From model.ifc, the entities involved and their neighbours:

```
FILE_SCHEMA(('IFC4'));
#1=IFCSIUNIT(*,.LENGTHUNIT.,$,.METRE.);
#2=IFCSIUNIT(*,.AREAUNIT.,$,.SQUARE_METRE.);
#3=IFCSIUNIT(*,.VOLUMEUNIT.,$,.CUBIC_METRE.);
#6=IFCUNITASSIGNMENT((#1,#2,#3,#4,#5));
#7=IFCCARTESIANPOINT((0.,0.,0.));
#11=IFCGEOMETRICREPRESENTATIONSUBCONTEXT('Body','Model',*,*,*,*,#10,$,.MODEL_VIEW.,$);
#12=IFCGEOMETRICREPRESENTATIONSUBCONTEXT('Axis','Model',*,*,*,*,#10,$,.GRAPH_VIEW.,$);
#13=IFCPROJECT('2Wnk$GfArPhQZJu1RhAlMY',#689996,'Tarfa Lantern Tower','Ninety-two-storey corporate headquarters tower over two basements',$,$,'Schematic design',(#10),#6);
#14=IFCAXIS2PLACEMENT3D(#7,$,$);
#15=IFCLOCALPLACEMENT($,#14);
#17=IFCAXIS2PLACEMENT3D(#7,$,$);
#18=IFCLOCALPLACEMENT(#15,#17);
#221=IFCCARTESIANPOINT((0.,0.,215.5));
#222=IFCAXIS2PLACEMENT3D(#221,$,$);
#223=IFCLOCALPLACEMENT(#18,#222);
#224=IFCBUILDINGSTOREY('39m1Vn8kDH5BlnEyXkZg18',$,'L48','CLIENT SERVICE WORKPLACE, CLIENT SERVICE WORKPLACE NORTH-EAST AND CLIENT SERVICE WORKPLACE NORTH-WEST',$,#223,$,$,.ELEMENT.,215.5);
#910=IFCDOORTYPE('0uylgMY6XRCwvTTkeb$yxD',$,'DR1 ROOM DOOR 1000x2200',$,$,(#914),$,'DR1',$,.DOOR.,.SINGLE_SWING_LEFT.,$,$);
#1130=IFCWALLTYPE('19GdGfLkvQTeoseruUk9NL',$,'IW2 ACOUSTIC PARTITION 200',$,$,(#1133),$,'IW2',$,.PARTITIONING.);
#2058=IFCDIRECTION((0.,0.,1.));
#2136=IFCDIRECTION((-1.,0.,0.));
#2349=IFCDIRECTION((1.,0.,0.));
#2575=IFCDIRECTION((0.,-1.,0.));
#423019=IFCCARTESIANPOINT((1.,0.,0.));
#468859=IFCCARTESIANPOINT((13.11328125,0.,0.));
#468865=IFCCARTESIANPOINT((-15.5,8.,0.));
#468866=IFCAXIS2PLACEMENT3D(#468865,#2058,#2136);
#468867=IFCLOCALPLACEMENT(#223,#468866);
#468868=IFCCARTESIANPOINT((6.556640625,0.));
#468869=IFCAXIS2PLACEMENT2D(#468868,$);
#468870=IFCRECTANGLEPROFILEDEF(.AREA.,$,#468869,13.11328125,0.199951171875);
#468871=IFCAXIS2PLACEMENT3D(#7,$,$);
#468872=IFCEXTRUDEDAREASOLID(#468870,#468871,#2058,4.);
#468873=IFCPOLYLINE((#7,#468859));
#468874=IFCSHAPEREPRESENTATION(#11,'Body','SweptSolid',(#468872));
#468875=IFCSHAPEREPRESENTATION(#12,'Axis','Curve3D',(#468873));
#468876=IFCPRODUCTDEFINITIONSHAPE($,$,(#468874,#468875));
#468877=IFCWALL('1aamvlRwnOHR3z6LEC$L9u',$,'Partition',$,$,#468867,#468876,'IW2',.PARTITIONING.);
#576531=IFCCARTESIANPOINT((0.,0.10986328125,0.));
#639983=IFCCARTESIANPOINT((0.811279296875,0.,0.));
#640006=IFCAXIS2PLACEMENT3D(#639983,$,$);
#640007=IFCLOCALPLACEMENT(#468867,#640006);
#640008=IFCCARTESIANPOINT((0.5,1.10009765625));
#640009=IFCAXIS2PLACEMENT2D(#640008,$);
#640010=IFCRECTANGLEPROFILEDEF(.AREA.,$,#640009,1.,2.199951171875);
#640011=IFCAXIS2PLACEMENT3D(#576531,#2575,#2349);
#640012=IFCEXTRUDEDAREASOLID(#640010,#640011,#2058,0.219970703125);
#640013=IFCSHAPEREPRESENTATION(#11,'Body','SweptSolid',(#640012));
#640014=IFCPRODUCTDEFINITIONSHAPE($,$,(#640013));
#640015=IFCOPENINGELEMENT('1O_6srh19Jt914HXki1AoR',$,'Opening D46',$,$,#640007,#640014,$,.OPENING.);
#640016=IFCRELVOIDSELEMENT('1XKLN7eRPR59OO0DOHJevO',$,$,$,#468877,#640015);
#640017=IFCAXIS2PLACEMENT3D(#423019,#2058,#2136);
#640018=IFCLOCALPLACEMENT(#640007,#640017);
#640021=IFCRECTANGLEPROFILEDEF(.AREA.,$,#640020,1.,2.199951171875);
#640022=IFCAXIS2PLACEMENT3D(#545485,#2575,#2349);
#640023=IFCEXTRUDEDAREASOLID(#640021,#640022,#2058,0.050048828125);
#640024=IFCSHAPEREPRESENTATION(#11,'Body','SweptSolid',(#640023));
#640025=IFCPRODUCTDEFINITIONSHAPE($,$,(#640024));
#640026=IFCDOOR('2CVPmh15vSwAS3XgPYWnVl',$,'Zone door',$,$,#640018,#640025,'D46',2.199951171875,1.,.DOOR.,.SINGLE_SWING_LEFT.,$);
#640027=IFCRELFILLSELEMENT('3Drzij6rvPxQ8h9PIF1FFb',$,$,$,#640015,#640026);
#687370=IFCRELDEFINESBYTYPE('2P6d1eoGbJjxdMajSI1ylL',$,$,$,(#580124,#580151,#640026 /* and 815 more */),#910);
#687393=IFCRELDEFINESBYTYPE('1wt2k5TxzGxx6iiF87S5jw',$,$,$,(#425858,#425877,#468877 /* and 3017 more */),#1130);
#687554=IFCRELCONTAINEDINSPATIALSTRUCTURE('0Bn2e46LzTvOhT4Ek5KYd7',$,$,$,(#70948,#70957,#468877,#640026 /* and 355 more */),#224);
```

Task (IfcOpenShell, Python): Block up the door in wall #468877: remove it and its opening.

```python
import ifcopenshell
import ifcopenshell.api.feature
import ifcopenshell.api.root
import ifcopenshell.geom
import ifcopenshell.util.shape

model = ifcopenshell.open("model.ifc")
settings = ifcopenshell.geom.settings()


def volume(element):
    """Net volume in cubic metres, openings subtracted."""
    shape = ifcopenshell.geom.create_shape(settings, element)
    return ifcopenshell.util.shape.get_volume(shape.geometry)


door = model.by_guid("2CVPmh15vSwAS3XgPYWnVl")
opening = door.FillsVoids[0].RelatingOpeningElement
wall = opening.VoidsElements[0].RelatingBuildingElement
before = volume(wall)

ifcopenshell.api.root.remove_product(model, product=door)
ifcopenshell.api.feature.remove_feature(model, feature=opening)

after = volume(wall)

print(f"wall volume {before:.3f} -> {after:.3f} m3")

model.write("model_v2.ifc")
```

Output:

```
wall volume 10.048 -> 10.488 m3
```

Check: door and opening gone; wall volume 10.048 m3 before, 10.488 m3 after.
